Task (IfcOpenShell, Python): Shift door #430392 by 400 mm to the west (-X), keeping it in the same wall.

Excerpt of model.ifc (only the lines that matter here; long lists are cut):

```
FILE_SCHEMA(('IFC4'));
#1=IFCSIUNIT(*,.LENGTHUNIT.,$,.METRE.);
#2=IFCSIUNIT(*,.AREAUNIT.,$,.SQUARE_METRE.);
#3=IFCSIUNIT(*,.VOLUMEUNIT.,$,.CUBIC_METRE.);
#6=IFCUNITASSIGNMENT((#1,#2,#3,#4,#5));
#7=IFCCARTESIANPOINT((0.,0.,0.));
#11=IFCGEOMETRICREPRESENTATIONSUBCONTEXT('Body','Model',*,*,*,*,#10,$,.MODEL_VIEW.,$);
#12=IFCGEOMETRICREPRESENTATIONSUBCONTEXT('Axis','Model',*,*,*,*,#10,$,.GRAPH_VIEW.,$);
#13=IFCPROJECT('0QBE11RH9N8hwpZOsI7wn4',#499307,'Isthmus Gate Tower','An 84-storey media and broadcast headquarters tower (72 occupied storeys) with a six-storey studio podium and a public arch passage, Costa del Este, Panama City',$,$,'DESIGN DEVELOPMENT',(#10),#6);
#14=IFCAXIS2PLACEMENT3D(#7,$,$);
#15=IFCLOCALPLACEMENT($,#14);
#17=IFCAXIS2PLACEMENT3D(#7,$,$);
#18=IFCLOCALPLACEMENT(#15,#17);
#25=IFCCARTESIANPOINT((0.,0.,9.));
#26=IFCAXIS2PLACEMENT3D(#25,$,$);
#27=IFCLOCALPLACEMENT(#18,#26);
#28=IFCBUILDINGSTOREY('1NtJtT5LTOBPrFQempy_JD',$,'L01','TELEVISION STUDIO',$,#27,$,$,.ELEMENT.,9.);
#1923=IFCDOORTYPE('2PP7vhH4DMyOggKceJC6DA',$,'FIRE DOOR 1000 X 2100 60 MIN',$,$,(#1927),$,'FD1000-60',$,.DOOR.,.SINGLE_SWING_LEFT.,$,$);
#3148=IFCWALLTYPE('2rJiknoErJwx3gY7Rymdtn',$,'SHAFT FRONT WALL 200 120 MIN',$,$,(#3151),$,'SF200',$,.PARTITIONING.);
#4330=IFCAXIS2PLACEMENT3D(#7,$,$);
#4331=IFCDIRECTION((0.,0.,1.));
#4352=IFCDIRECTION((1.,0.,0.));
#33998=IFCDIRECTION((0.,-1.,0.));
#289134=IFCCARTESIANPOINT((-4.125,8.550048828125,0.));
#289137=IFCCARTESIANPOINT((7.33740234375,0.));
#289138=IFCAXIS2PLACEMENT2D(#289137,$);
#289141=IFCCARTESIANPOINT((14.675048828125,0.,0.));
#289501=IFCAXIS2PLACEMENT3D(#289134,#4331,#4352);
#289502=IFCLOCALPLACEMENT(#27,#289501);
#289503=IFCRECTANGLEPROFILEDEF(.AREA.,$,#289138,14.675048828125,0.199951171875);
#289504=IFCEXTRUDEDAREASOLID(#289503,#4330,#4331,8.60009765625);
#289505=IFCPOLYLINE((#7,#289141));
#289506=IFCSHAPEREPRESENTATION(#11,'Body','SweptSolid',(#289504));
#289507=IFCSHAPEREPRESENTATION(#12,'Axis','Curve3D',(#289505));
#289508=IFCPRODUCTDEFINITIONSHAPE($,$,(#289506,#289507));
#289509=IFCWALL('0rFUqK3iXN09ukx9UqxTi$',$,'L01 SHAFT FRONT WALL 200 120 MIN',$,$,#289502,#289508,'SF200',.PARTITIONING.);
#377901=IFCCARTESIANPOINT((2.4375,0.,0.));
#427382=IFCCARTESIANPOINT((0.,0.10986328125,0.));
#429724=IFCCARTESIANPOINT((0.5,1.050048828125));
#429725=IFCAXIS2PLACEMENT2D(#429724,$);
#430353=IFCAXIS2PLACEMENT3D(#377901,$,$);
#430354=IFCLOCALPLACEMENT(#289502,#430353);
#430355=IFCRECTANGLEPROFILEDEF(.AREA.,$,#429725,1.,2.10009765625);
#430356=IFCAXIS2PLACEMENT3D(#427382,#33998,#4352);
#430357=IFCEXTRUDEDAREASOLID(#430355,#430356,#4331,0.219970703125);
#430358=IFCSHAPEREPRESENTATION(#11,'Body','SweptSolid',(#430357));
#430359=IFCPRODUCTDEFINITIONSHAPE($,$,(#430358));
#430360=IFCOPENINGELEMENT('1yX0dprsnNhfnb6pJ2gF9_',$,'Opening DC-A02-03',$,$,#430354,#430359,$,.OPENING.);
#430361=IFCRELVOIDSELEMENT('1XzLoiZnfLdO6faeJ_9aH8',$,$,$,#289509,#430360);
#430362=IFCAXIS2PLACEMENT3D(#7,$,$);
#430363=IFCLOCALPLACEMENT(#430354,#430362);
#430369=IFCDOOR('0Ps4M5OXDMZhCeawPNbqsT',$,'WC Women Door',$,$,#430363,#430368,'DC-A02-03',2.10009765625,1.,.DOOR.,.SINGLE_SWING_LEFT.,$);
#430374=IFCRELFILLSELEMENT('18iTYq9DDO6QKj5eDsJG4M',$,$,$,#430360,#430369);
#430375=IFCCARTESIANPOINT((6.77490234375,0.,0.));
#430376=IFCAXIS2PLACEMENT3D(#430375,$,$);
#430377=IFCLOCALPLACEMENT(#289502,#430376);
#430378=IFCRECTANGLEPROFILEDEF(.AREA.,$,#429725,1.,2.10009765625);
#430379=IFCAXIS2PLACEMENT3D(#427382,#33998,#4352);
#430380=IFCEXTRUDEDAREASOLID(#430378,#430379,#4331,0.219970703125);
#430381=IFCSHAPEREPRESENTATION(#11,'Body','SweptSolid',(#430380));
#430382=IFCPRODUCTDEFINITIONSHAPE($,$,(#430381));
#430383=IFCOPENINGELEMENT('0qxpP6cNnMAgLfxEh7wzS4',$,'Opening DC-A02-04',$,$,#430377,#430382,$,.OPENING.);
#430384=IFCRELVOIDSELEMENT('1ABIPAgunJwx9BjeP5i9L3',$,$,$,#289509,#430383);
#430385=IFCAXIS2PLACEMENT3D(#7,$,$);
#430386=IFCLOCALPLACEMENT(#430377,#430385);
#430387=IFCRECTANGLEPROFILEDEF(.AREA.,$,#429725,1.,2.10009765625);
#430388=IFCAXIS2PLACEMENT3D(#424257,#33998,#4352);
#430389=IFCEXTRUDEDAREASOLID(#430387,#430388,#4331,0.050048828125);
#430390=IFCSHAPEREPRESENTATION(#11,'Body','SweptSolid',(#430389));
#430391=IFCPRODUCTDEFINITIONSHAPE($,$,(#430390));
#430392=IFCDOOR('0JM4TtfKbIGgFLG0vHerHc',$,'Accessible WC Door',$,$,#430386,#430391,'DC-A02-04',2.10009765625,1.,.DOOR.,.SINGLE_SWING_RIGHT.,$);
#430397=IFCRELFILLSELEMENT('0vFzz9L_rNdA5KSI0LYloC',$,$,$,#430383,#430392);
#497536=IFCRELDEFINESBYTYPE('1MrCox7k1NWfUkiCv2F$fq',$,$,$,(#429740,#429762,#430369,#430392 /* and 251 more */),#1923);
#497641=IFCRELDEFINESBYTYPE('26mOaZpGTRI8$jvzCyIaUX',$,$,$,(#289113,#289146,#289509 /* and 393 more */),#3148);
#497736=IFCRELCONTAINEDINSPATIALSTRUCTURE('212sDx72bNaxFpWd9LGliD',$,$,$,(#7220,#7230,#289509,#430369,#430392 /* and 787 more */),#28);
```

```python
import ifcopenshell
import ifcopenshell.api.geometry
import ifcopenshell.util.placement
import ifcopenshell.util.unit

model = ifcopenshell.open("model.ifc")
unit_scale = ifcopenshell.util.unit.calculate_unit_scale(model)

door = model.by_guid("0JM4TtfKbIGgFLG0vHerHc")
opening = door.FillsVoids[0].RelatingOpeningElement
wall = opening.VoidsElements[0].RelatingBuildingElement

wall_matrix = ifcopenshell.util.placement.get_local_placement(wall.ObjectPlacement)
shift = wall_matrix[:3, 0] * -0.4 / unit_scale
before = ifcopenshell.util.placement.get_local_placement(door.ObjectPlacement)[:3, 3].copy()

# The door is placed relative to its opening, so it follows when the opening moves.
matrix = ifcopenshell.util.placement.get_local_placement(opening.ObjectPlacement)
matrix[:3, 3] += shift
ifcopenshell.api.geometry.edit_object_placement(
    model, product=opening, matrix=matrix, is_si=False, should_transform_children=True
)

after = ifcopenshell.util.placement.get_local_placement(door.ObjectPlacement)[:3, 3]
print("door moved by", (after - before).round(3) + 0.0)

model.write("model_updated.ifc")
```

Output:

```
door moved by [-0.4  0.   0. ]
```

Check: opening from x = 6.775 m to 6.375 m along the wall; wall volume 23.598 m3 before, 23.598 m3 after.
